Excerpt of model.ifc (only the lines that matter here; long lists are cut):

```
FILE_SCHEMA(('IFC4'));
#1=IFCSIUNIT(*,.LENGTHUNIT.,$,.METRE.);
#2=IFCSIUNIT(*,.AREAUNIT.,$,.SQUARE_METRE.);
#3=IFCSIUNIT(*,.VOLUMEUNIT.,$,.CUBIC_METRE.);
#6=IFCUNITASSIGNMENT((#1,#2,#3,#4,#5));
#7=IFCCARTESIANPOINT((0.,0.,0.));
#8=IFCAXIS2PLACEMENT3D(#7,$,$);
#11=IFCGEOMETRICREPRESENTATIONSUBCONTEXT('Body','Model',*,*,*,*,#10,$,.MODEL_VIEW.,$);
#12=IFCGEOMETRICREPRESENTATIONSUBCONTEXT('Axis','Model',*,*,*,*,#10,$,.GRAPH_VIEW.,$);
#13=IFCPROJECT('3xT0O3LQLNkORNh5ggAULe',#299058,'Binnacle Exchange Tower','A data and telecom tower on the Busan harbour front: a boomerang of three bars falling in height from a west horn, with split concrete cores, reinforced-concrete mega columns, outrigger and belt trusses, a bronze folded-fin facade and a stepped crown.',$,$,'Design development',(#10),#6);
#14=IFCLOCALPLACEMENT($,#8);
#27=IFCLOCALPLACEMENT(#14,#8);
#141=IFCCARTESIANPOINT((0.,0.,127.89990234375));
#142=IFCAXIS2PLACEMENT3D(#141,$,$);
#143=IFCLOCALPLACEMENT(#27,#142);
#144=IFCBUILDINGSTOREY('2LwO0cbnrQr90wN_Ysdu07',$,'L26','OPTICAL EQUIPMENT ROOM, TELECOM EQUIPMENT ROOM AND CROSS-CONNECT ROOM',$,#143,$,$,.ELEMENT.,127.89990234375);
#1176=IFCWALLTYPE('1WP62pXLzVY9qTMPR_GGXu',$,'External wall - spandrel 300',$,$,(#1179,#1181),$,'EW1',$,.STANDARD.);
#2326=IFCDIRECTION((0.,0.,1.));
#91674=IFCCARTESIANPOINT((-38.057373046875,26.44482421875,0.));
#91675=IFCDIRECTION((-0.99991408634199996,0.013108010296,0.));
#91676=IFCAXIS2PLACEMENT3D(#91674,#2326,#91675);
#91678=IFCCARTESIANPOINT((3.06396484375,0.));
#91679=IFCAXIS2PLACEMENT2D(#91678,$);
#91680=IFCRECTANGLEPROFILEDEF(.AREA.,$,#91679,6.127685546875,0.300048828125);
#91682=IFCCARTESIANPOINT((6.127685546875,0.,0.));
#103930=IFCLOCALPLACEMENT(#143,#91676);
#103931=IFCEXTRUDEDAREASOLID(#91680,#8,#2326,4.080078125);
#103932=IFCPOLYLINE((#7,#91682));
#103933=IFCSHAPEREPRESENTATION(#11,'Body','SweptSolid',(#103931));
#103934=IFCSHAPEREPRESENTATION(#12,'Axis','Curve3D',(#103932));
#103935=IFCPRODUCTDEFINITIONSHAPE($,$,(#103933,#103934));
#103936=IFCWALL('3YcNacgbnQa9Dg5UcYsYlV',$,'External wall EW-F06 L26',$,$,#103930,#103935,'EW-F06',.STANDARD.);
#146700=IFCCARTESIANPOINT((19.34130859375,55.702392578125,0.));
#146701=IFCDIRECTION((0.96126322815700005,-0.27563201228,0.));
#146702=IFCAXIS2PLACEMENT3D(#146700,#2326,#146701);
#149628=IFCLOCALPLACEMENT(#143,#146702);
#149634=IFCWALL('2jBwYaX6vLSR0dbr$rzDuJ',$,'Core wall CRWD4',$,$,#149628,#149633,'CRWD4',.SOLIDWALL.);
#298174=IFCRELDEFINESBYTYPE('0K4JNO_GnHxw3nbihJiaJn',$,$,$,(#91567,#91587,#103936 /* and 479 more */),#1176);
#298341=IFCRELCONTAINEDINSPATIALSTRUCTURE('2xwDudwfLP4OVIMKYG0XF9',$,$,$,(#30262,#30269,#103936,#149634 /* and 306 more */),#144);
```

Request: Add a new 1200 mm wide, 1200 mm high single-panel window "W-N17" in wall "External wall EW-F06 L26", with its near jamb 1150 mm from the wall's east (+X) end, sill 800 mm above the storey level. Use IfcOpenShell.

```python
import numpy as np
import ifcopenshell
import ifcopenshell.api.feature
import ifcopenshell.api.geometry
import ifcopenshell.api.root
import ifcopenshell.api.spatial
import ifcopenshell.geom
import ifcopenshell.util.element
import ifcopenshell.util.placement
import ifcopenshell.util.representation
import ifcopenshell.util.shape
import ifcopenshell.util.unit

model = ifcopenshell.open("model.ifc")
unit_scale = ifcopenshell.util.unit.calculate_unit_scale(model)
settings = ifcopenshell.geom.settings()


def volume(element):
    """Net volume in cubic metres, openings subtracted."""
    shape = ifcopenshell.geom.create_shape(settings, element)
    return ifcopenshell.util.shape.get_volume(shape.geometry)


wall = model.by_guid("3YcNacgbnQa9Dg5UcYsYlV")
storey = ifcopenshell.util.element.get_container(wall, ifc_class="IfcBuildingStorey")
context = ifcopenshell.util.representation.get_context(model, "Model", "Body", "MODEL_VIEW")
before = volume(wall)

width, height, from_end, sill = 1.2, 1.2, 1.15, 0.8  # metres

# The wall runs along its own X axis, and the end named is its -X end.
wall_shape = ifcopenshell.geom.create_shape(settings, wall)
x, y, z = ifcopenshell.util.shape.get_vertices(wall_shape.geometry).T
start = x.min() + from_end
face, thickness = float(y.min()), float(y.max() - y.min())
wall_matrix = ifcopenshell.util.placement.get_local_placement(wall.ObjectPlacement)
level = ifcopenshell.util.placement.get_local_placement(storey.ObjectPlacement)[2, 3]


def in_wall(x, y):
    """Placement at x, y metres in the wall's axes, at sill height."""
    matrix = wall_matrix.copy()
    matrix[:, 3] = wall_matrix @ np.array([x / unit_scale, y / unit_scale, 0.0, 1.0])
    matrix[2, 3] = level + sill / unit_scale
    return matrix


# Opening: a box that overshoots both wall faces by 50 mm.
opening = ifcopenshell.api.root.create_entity(model, ifc_class="IfcOpeningElement", predefined_type="OPENING")
box = ifcopenshell.api.geometry.add_wall_representation(
    model, context=context, length=width, height=height, thickness=thickness + 0.1
)
ifcopenshell.api.geometry.assign_representation(model, product=opening, representation=box)
ifcopenshell.api.geometry.edit_object_placement(model, product=opening, matrix=in_wall(start, face - 0.05), is_si=False)
ifcopenshell.api.feature.add_feature(model, feature=opening, element=wall)

window = ifcopenshell.api.root.create_entity(model, ifc_class="IfcWindow", name="W-N17", predefined_type="WINDOW")
window.OverallWidth, window.OverallHeight = width / unit_scale, height / unit_scale
window.PartitioningType = "SINGLE_PANEL"
body = ifcopenshell.api.geometry.add_window_representation(
    model,
    context=context,
    overall_width=window.OverallWidth,
    overall_height=window.OverallHeight,
    partition_type="SINGLE_PANEL",
)
ifcopenshell.api.geometry.assign_representation(model, product=window, representation=body)
ifcopenshell.api.spatial.assign_container(model, products=[window], relating_structure=storey)
ifcopenshell.api.feature.add_filling(model, opening=opening, element=window)

# Centre the window in the wall's thickness.
ifcopenshell.api.geometry.edit_object_placement(model, product=window, matrix=in_wall(start, face), is_si=False)
window_shape = ifcopenshell.geom.create_shape(settings, window)
depth = ifcopenshell.util.shape.get_vertices(window_shape.geometry)[:, 1]
offset = face + thickness / 2 - (depth.min() + depth.max()) / 2
ifcopenshell.api.geometry.edit_object_placement(model, product=window, matrix=in_wall(start, offset), is_si=False)

after = volume(wall)

print(f"wall volume {before:.3f} -> {after:.3f} m3")

model.write("model_updated.ifc")
```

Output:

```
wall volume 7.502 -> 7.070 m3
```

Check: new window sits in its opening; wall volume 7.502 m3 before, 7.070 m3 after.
